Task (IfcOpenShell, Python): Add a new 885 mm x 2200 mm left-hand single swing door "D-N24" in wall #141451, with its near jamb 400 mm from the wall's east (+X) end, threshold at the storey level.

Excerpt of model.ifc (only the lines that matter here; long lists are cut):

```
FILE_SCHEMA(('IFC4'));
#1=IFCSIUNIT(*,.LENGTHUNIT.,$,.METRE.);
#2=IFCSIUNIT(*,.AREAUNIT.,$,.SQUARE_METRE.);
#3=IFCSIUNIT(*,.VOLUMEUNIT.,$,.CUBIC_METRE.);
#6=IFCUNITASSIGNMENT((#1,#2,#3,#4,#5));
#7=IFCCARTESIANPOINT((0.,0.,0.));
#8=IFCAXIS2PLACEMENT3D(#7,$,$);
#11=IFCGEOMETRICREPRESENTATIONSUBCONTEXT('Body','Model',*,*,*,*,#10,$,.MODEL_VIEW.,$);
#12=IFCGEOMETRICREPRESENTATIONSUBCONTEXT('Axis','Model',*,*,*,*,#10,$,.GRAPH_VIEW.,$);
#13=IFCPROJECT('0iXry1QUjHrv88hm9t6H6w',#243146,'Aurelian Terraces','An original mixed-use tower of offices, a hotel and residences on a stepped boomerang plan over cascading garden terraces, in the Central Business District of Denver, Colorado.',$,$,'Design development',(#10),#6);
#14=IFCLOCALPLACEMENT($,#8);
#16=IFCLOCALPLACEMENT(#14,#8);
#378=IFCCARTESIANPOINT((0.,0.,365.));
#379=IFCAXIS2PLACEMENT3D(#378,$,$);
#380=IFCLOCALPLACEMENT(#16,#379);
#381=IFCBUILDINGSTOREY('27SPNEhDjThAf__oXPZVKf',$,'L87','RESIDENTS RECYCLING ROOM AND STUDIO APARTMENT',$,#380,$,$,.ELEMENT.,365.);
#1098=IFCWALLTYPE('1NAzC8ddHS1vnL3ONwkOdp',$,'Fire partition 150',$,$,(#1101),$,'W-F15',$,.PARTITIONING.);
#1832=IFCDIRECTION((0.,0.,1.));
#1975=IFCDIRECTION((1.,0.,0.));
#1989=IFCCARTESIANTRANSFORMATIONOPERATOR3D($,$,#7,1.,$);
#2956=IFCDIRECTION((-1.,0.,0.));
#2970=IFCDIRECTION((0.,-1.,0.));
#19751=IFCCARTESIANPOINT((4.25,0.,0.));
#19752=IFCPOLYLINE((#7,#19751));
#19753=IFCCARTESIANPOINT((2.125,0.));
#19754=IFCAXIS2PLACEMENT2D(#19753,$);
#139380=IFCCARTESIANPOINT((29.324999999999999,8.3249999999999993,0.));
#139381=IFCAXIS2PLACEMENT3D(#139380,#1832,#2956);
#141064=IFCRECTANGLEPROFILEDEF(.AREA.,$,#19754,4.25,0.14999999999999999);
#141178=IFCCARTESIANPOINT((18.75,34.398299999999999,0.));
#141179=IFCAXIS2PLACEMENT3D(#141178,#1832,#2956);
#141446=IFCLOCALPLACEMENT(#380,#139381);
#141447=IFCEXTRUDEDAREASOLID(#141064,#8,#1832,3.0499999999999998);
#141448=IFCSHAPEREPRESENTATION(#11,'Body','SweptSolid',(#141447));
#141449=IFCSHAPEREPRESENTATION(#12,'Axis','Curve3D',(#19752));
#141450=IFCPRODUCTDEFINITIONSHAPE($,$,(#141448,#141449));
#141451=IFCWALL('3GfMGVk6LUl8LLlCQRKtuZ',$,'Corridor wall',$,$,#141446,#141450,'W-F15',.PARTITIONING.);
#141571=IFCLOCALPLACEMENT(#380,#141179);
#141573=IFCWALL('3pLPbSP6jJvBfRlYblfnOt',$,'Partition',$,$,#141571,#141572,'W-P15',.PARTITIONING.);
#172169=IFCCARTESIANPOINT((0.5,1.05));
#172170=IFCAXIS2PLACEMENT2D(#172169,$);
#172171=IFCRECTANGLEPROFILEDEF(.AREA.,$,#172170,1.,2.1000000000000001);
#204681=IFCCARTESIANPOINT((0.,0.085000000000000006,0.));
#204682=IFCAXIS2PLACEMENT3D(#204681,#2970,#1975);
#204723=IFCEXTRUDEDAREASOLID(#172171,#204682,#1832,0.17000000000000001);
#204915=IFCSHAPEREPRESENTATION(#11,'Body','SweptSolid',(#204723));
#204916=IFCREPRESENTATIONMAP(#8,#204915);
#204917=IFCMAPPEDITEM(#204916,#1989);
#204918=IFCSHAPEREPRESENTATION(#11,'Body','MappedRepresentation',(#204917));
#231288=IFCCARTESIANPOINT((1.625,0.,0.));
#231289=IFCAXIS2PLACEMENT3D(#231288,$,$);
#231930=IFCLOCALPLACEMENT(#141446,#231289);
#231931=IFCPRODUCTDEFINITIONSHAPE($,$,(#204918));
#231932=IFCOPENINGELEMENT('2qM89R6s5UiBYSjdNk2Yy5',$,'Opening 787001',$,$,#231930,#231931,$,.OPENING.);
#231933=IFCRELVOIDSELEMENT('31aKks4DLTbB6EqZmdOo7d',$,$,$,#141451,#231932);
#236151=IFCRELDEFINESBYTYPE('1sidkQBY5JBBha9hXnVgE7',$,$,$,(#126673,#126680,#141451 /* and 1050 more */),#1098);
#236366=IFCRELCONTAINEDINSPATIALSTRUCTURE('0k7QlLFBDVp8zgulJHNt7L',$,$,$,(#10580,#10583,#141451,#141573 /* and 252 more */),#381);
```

```python
import numpy as np
import ifcopenshell
import ifcopenshell.api.feature
import ifcopenshell.api.geometry
import ifcopenshell.api.root
import ifcopenshell.api.spatial
import ifcopenshell.geom
import ifcopenshell.util.element
import ifcopenshell.util.placement
import ifcopenshell.util.representation
import ifcopenshell.util.shape
import ifcopenshell.util.unit

model = ifcopenshell.open("model.ifc")
unit_scale = ifcopenshell.util.unit.calculate_unit_scale(model)
settings = ifcopenshell.geom.settings()


def volume(element):
    """Net volume in cubic metres, openings subtracted."""
    shape = ifcopenshell.geom.create_shape(settings, element)
    return ifcopenshell.util.shape.get_volume(shape.geometry)


wall = model.by_guid("3GfMGVk6LUl8LLlCQRKtuZ")
storey = ifcopenshell.util.element.get_container(wall, ifc_class="IfcBuildingStorey")
context = ifcopenshell.util.representation.get_context(model, "Model", "Body", "MODEL_VIEW")
before = volume(wall)

width, height, from_end, sill = 0.885, 2.2, 0.4, 0.0  # metres

# The wall runs along its own X axis, and the end named is its -X end.
wall_shape = ifcopenshell.geom.create_shape(settings, wall)
x, y, z = ifcopenshell.util.shape.get_vertices(wall_shape.geometry).T
start = x.min() + from_end
face, thickness = float(y.min()), float(y.max() - y.min())
wall_matrix = ifcopenshell.util.placement.get_local_placement(wall.ObjectPlacement)
level = ifcopenshell.util.placement.get_local_placement(storey.ObjectPlacement)[2, 3]


def in_wall(x, y):
    """Placement at x, y metres in the wall's axes, at sill height."""
    matrix = wall_matrix.copy()
    matrix[:, 3] = wall_matrix @ np.array([x / unit_scale, y / unit_scale, 0.0, 1.0])
    matrix[2, 3] = level + sill / unit_scale
    return matrix


# Opening: a box that overshoots both wall faces by 50 mm.
opening = ifcopenshell.api.root.create_entity(model, ifc_class="IfcOpeningElement", predefined_type="OPENING")
box = ifcopenshell.api.geometry.add_wall_representation(
    model, context=context, length=width, height=height, thickness=thickness + 0.1
)
ifcopenshell.api.geometry.assign_representation(model, product=opening, representation=box)
ifcopenshell.api.geometry.edit_object_placement(model, product=opening, matrix=in_wall(start, face - 0.05), is_si=False)
ifcopenshell.api.feature.add_feature(model, feature=opening, element=wall)

door = ifcopenshell.api.root.create_entity(model, ifc_class="IfcDoor", name="D-N24", predefined_type="DOOR")
door.OverallWidth, door.OverallHeight = width / unit_scale, height / unit_scale
door.OperationType = "SINGLE_SWING_LEFT"
body = ifcopenshell.api.geometry.add_door_representation(
    model,
    context=context,
    overall_width=door.OverallWidth,
    overall_height=door.OverallHeight,
    operation_type="SINGLE_SWING_LEFT",
    lining_properties={"LiningDepth": thickness / unit_scale, "ThresholdDepth": thickness / unit_scale},
)
ifcopenshell.api.geometry.assign_representation(model, product=door, representation=body)
ifcopenshell.api.spatial.assign_container(model, products=[door], relating_structure=storey)
ifcopenshell.api.feature.add_filling(model, opening=opening, element=door)

# The lining spans the wall, so the door starts at the wall face.
ifcopenshell.api.geometry.edit_object_placement(model, product=door, matrix=in_wall(start, face), is_si=False)

after = volume(wall)

print(f"wall volume {before:.3f} -> {after:.3f} m3")

model.write("model_edited.ifc")
```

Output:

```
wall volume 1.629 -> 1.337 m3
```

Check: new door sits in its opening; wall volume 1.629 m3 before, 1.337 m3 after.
